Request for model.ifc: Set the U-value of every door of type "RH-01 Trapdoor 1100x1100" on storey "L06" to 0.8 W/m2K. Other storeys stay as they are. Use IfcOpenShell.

First a look at what the model holds.

```python
import ifcopenshell
import ifcopenshell.util.element

model = ifcopenshell.open("model.ifc")
print(model.schema)
storey = next(s for s in model.by_type("IfcBuildingStorey") if s.Name == "L06")
doors = [e for e in ifcopenshell.util.element.get_decomposition(storey) if e.is_a("IfcDoor")]
seen = {}
for e in doors:
    element_type = ifcopenshell.util.element.get_type(e)
    key = (element_type.Name if element_type != e and element_type else None, ifcopenshell.util.element.get_pset(e, "Pset_DoorCommon", "ThermalTransmittance"))
    seen[key] = seen.get(key, 0) + 1
for (name, value), count in sorted(seen.items(), key=str):
    print(count, "x", name, "|", value)
```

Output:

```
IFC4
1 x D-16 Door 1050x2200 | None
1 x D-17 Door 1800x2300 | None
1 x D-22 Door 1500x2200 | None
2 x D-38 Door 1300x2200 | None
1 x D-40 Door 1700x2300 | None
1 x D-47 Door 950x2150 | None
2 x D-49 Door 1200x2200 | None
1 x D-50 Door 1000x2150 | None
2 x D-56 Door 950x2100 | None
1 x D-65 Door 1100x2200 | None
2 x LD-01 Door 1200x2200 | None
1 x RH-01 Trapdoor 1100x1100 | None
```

```python
import ifcopenshell
import ifcopenshell.api.pset
import ifcopenshell.util.element

model = ifcopenshell.open("model.ifc")

storey = next(s for s in model.by_type("IfcBuildingStorey") if s.Name == "L06")
doors = [e for e in ifcopenshell.util.element.get_decomposition(storey) if e.is_a("IfcDoor")]

count = 0
for e in doors:
    element_type = ifcopenshell.util.element.get_type(e)
    if element_type in (None, e) or element_type.Name != "RH-01 Trapdoor 1100x1100":
        continue
    # add_pset returns the element's existing set when there is one.
    pset = ifcopenshell.api.pset.add_pset(model, product=e, name="Pset_DoorCommon")
    ifcopenshell.api.pset.edit_pset(model, pset=pset, properties={"ThermalTransmittance": 0.8})
    count += 1

print(count, "doors updated")

model.write("model_rev.ifc")
```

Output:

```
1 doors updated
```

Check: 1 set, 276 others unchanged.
